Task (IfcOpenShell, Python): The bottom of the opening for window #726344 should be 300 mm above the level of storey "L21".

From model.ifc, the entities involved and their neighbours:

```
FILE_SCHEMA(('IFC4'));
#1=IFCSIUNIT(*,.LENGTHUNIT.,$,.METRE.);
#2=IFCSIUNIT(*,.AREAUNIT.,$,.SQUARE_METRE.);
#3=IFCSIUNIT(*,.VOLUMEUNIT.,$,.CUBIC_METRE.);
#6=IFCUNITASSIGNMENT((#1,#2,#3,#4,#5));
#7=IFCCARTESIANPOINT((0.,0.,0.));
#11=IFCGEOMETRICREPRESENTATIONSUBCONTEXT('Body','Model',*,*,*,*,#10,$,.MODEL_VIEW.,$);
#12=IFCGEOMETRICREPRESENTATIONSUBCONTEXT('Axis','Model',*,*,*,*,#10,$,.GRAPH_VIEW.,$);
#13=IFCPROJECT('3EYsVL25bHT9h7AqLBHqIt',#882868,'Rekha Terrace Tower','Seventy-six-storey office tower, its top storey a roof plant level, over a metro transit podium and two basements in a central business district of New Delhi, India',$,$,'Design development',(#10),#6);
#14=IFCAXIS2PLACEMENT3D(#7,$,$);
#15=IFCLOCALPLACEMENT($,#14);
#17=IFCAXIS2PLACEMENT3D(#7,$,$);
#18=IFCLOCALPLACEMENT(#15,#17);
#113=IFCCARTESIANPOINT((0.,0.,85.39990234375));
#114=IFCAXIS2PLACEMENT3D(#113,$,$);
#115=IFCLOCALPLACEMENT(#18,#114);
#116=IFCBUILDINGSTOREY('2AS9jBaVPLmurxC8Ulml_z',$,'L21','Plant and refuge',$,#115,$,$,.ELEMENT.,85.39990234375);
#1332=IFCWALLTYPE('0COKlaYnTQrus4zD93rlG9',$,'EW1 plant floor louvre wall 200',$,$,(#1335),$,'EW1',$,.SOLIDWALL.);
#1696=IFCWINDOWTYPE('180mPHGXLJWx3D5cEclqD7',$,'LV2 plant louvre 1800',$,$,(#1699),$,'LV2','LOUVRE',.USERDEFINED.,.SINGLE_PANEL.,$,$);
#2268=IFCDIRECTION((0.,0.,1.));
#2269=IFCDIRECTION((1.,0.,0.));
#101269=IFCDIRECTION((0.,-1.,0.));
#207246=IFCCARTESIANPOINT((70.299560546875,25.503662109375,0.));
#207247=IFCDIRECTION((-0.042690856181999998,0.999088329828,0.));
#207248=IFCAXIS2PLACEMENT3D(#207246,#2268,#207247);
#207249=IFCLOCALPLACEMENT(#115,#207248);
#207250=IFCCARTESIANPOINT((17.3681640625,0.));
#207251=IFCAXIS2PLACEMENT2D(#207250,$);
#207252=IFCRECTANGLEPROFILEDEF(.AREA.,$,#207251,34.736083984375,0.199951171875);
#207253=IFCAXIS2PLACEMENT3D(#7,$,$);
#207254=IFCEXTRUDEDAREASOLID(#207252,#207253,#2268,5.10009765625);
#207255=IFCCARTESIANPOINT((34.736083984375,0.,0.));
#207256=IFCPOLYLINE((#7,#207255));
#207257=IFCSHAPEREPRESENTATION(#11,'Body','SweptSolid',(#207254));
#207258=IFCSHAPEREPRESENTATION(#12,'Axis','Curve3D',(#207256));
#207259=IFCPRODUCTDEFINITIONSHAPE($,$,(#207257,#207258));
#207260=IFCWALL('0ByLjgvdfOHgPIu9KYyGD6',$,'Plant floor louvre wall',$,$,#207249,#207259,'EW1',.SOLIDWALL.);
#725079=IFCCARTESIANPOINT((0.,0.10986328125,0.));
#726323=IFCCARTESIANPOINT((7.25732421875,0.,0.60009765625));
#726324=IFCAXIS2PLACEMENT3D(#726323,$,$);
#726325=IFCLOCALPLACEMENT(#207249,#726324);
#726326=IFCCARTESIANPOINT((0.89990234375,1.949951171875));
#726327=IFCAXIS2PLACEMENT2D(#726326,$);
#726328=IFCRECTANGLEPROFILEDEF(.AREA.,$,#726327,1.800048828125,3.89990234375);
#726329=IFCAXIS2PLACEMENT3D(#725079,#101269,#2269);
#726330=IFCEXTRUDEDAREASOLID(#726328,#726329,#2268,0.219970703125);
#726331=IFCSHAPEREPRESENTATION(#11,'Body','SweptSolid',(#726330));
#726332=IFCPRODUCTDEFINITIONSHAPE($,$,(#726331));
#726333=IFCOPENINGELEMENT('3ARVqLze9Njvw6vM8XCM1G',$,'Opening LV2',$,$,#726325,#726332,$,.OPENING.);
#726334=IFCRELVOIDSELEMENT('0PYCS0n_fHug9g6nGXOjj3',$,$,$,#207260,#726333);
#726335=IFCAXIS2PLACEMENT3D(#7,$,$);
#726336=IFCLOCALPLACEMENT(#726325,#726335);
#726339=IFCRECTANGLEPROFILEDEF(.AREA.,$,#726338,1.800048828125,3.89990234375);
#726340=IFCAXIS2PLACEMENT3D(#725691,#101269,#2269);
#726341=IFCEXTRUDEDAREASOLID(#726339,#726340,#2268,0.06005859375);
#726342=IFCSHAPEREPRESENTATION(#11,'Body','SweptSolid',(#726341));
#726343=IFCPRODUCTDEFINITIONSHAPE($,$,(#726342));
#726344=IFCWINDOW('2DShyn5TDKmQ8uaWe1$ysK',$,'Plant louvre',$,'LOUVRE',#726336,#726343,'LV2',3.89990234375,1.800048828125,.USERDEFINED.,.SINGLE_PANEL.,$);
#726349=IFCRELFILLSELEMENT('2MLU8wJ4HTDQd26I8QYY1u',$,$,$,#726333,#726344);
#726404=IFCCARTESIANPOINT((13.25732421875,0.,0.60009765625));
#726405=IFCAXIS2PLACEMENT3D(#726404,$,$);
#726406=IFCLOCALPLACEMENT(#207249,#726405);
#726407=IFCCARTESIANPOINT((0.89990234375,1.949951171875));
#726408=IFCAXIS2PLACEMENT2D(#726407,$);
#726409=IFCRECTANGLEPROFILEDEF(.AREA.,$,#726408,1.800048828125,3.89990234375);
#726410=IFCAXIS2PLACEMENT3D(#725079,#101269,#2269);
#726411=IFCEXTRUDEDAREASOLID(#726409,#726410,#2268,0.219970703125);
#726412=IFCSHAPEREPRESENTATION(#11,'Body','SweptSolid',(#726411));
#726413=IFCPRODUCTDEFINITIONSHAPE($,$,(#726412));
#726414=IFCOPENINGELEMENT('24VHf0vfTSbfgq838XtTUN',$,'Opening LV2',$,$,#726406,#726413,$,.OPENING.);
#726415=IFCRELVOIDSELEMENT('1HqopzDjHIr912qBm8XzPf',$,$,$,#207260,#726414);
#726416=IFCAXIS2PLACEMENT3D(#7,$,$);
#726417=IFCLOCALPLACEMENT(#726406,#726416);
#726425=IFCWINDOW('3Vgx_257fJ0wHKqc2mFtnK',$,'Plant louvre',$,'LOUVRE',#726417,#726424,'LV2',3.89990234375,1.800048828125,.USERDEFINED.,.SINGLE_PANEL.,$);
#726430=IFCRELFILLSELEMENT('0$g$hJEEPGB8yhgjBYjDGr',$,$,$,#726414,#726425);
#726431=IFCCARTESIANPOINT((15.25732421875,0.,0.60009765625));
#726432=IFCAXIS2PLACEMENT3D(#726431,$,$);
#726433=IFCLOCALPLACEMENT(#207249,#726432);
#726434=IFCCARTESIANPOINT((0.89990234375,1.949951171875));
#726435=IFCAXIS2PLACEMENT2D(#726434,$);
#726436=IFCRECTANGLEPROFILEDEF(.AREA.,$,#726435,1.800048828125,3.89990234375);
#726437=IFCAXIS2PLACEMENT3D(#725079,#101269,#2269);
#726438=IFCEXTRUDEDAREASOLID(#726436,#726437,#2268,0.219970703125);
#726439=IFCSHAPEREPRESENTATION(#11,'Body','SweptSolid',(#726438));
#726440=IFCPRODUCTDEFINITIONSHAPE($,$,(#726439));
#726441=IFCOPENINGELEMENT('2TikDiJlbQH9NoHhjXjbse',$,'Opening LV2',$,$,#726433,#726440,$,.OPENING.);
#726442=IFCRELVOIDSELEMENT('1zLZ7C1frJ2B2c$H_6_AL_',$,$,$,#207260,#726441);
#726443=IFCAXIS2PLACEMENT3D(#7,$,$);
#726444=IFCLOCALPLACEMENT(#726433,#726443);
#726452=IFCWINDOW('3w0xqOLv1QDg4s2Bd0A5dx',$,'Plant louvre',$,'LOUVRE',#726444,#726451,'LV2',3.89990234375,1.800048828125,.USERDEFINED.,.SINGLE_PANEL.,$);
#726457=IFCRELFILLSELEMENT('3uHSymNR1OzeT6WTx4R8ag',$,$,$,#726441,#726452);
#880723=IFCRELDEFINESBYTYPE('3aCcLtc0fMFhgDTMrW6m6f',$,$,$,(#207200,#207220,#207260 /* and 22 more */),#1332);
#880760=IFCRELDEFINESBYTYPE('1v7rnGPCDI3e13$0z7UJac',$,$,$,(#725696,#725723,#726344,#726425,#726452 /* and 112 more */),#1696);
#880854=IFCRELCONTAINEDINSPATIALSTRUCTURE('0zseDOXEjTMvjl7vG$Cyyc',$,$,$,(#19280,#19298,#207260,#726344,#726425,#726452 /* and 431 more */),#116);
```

```python
import numpy as np
import ifcopenshell
import ifcopenshell.api.geometry
import ifcopenshell.geom
import ifcopenshell.util.element
import ifcopenshell.util.placement
import ifcopenshell.util.shape
import ifcopenshell.util.unit

model = ifcopenshell.open("model.ifc")
unit_scale = ifcopenshell.util.unit.calculate_unit_scale(model)

window = model.by_guid("2DShyn5TDKmQ8uaWe1$ysK")
opening = window.FillsVoids[0].RelatingOpeningElement
storey = ifcopenshell.util.element.get_container(window, ifc_class="IfcBuildingStorey")
level = ifcopenshell.util.placement.get_local_placement(storey.ObjectPlacement)[2, 3]

# The opening's origin need not be at the sill, so measure its lowest point.
shape = ifcopenshell.geom.create_shape(ifcopenshell.geom.settings(), opening)
bottom = ifcopenshell.util.shape.get_shape_bottom_elevation(shape, shape.geometry) / unit_scale
dz = level + 0.3 / unit_scale - bottom

shift = np.array([0.0, 0.0, dz])
# The window is placed relative to its opening, so it follows when the opening moves.
matrix = ifcopenshell.util.placement.get_local_placement(opening.ObjectPlacement)
matrix[:3, 3] += shift
ifcopenshell.api.geometry.edit_object_placement(
    model, product=opening, matrix=matrix, is_si=False, should_transform_children=True
)

print(f"moved by {dz * unit_scale:+.3f} m")

model.write("model_v2.ifc")
```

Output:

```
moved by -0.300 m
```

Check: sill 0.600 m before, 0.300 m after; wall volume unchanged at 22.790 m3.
